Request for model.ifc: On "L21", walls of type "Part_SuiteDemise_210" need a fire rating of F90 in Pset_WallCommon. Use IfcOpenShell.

First a look at what the model holds.

```python
import ifcopenshell
import ifcopenshell.util.element

model = ifcopenshell.open("model.ifc")
print(model.schema)
storey = next(s for s in model.by_type("IfcBuildingStorey") if s.Name == "L21")
walls = [e for e in ifcopenshell.util.element.get_decomposition(storey) if e.is_a("IfcWall")]
seen = {}
for e in walls:
    element_type = ifcopenshell.util.element.get_type(e)
    key = (element_type.Name if element_type != e and element_type else None, ifcopenshell.util.element.get_pset(e, "Pset_WallCommon", "FireRating"))
    seen[key] = seen.get(key, 0) + 1
for (name, value), count in sorted(seen.items(), key=str):
    print(count, "x", name, "|", value)
```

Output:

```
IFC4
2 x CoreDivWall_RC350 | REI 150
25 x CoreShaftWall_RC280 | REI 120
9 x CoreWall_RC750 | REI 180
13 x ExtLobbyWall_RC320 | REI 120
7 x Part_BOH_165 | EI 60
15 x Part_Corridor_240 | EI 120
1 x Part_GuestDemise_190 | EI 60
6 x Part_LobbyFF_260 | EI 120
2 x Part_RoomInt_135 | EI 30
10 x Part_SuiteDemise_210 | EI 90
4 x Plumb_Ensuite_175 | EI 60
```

```python
import ifcopenshell
import ifcopenshell.api.pset
import ifcopenshell.util.element

model = ifcopenshell.open("model.ifc")

storey = next(s for s in model.by_type("IfcBuildingStorey") if s.Name == "L21")
walls = [e for e in ifcopenshell.util.element.get_decomposition(storey) if e.is_a("IfcWall")]

count = 0
for e in walls:
    element_type = ifcopenshell.util.element.get_type(e)
    if element_type in (None, e) or element_type.Name != "Part_SuiteDemise_210":
        continue
    found = ifcopenshell.util.element.get_pset(e, "Pset_WallCommon", should_inherit=False)
    if found:
        pset = model.by_id(found["id"])
        if len(ifcopenshell.util.element.get_elements_by_pset(pset)) > 1:
            pset = ifcopenshell.api.pset.unshare_pset(model, products=[e], pset=pset)[0]
    else:
        pset = ifcopenshell.api.pset.add_pset(model, product=e, name="Pset_WallCommon")
    ifcopenshell.api.pset.edit_pset(model, pset=pset, properties={"FireRating": "F90"})
    count += 1

print(count, "walls updated")

model.write("model_edited.ifc")
```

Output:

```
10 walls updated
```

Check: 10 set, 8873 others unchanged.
